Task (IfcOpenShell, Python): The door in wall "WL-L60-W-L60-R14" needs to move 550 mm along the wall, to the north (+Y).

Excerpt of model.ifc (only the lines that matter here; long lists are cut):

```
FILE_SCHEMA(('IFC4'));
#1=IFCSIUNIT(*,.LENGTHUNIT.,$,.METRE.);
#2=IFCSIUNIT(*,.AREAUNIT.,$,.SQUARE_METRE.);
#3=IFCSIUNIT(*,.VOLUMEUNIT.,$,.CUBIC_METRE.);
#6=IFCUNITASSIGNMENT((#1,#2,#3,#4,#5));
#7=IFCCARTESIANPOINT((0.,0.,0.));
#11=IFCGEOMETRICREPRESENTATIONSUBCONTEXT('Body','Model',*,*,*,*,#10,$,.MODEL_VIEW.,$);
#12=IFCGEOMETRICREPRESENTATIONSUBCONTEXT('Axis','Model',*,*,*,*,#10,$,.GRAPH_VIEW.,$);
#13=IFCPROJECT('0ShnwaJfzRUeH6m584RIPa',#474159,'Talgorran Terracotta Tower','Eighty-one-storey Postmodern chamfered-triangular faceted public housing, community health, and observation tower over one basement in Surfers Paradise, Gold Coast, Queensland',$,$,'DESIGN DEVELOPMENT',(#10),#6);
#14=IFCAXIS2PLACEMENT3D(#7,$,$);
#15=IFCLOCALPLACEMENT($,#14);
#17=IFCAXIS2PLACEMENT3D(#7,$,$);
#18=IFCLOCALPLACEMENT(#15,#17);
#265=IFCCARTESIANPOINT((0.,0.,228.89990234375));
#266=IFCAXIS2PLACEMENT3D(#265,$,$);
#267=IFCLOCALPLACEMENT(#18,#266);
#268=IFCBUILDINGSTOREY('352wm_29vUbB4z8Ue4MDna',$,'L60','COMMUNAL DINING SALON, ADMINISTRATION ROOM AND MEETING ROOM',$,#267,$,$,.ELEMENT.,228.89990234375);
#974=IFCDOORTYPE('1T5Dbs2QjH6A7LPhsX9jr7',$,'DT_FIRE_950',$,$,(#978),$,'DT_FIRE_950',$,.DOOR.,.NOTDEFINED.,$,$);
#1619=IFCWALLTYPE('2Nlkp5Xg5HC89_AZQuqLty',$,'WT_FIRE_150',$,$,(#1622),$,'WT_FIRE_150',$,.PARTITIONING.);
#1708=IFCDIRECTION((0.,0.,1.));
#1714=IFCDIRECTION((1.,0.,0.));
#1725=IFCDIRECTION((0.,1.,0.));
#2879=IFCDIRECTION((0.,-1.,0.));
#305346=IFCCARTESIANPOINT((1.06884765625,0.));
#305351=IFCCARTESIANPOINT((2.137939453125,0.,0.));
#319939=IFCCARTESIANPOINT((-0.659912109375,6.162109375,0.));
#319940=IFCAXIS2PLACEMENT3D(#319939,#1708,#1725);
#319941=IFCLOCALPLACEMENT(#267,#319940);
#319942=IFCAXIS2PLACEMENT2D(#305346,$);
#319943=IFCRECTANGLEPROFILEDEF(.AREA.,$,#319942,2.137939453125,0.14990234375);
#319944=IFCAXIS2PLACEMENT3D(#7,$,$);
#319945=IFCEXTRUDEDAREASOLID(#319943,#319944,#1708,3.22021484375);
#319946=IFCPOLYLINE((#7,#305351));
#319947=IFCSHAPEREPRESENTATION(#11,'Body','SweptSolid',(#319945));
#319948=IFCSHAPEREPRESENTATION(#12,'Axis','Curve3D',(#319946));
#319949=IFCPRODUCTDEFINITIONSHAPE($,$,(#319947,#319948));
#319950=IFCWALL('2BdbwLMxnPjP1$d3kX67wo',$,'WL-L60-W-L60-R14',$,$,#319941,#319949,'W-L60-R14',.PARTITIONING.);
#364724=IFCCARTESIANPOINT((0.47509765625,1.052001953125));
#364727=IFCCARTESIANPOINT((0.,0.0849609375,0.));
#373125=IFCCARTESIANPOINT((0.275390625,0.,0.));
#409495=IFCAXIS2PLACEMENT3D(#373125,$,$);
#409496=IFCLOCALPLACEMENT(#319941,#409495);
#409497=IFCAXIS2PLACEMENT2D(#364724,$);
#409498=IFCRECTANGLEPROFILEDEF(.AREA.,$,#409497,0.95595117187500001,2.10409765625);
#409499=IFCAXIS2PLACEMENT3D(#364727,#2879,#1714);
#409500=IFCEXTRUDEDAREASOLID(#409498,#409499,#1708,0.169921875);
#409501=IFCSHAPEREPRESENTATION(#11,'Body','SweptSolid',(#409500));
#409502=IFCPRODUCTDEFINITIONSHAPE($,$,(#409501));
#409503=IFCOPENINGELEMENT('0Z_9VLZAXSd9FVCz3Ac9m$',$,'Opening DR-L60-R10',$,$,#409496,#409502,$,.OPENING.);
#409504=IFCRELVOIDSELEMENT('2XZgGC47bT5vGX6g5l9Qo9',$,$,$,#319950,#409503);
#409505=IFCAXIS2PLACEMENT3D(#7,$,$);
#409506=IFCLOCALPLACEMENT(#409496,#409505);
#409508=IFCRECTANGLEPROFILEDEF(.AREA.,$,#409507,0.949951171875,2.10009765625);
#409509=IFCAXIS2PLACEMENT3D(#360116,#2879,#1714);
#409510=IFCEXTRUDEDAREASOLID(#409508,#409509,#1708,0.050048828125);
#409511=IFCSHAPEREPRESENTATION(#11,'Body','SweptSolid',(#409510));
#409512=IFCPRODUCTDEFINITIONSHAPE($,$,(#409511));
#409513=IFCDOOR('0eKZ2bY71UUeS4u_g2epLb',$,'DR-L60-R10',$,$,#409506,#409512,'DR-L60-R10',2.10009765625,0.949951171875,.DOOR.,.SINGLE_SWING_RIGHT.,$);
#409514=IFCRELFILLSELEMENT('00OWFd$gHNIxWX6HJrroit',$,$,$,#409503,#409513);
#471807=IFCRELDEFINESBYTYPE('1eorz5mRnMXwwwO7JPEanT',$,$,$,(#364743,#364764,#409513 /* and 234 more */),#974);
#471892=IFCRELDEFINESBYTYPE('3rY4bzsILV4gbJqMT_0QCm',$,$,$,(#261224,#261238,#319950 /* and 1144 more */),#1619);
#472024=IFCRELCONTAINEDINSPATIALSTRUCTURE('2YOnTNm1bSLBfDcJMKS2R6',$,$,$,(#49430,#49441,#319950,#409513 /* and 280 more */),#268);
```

```python
import ifcopenshell
import ifcopenshell.api.geometry
import ifcopenshell.util.placement
import ifcopenshell.util.unit

model = ifcopenshell.open("model.ifc")
unit_scale = ifcopenshell.util.unit.calculate_unit_scale(model)

door = model.by_id(409513)
opening = door.FillsVoids[0].RelatingOpeningElement
wall = opening.VoidsElements[0].RelatingBuildingElement

wall_matrix = ifcopenshell.util.placement.get_local_placement(wall.ObjectPlacement)
shift = wall_matrix[:3, 0] * 0.55 / unit_scale
before = ifcopenshell.util.placement.get_local_placement(door.ObjectPlacement)[:3, 3].copy()

# The door is placed relative to its opening, so it follows when the opening moves.
matrix = ifcopenshell.util.placement.get_local_placement(opening.ObjectPlacement)
matrix[:3, 3] += shift
ifcopenshell.api.geometry.edit_object_placement(
    model, product=opening, matrix=matrix, is_si=False, should_transform_children=True
)

after = ifcopenshell.util.placement.get_local_placement(door.ObjectPlacement)[:3, 3]
print("door moved by", (after - before).round(3) + 0.0)

model.write("model-out.ifc")
```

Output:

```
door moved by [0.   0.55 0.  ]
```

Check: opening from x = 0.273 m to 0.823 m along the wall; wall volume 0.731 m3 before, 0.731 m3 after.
